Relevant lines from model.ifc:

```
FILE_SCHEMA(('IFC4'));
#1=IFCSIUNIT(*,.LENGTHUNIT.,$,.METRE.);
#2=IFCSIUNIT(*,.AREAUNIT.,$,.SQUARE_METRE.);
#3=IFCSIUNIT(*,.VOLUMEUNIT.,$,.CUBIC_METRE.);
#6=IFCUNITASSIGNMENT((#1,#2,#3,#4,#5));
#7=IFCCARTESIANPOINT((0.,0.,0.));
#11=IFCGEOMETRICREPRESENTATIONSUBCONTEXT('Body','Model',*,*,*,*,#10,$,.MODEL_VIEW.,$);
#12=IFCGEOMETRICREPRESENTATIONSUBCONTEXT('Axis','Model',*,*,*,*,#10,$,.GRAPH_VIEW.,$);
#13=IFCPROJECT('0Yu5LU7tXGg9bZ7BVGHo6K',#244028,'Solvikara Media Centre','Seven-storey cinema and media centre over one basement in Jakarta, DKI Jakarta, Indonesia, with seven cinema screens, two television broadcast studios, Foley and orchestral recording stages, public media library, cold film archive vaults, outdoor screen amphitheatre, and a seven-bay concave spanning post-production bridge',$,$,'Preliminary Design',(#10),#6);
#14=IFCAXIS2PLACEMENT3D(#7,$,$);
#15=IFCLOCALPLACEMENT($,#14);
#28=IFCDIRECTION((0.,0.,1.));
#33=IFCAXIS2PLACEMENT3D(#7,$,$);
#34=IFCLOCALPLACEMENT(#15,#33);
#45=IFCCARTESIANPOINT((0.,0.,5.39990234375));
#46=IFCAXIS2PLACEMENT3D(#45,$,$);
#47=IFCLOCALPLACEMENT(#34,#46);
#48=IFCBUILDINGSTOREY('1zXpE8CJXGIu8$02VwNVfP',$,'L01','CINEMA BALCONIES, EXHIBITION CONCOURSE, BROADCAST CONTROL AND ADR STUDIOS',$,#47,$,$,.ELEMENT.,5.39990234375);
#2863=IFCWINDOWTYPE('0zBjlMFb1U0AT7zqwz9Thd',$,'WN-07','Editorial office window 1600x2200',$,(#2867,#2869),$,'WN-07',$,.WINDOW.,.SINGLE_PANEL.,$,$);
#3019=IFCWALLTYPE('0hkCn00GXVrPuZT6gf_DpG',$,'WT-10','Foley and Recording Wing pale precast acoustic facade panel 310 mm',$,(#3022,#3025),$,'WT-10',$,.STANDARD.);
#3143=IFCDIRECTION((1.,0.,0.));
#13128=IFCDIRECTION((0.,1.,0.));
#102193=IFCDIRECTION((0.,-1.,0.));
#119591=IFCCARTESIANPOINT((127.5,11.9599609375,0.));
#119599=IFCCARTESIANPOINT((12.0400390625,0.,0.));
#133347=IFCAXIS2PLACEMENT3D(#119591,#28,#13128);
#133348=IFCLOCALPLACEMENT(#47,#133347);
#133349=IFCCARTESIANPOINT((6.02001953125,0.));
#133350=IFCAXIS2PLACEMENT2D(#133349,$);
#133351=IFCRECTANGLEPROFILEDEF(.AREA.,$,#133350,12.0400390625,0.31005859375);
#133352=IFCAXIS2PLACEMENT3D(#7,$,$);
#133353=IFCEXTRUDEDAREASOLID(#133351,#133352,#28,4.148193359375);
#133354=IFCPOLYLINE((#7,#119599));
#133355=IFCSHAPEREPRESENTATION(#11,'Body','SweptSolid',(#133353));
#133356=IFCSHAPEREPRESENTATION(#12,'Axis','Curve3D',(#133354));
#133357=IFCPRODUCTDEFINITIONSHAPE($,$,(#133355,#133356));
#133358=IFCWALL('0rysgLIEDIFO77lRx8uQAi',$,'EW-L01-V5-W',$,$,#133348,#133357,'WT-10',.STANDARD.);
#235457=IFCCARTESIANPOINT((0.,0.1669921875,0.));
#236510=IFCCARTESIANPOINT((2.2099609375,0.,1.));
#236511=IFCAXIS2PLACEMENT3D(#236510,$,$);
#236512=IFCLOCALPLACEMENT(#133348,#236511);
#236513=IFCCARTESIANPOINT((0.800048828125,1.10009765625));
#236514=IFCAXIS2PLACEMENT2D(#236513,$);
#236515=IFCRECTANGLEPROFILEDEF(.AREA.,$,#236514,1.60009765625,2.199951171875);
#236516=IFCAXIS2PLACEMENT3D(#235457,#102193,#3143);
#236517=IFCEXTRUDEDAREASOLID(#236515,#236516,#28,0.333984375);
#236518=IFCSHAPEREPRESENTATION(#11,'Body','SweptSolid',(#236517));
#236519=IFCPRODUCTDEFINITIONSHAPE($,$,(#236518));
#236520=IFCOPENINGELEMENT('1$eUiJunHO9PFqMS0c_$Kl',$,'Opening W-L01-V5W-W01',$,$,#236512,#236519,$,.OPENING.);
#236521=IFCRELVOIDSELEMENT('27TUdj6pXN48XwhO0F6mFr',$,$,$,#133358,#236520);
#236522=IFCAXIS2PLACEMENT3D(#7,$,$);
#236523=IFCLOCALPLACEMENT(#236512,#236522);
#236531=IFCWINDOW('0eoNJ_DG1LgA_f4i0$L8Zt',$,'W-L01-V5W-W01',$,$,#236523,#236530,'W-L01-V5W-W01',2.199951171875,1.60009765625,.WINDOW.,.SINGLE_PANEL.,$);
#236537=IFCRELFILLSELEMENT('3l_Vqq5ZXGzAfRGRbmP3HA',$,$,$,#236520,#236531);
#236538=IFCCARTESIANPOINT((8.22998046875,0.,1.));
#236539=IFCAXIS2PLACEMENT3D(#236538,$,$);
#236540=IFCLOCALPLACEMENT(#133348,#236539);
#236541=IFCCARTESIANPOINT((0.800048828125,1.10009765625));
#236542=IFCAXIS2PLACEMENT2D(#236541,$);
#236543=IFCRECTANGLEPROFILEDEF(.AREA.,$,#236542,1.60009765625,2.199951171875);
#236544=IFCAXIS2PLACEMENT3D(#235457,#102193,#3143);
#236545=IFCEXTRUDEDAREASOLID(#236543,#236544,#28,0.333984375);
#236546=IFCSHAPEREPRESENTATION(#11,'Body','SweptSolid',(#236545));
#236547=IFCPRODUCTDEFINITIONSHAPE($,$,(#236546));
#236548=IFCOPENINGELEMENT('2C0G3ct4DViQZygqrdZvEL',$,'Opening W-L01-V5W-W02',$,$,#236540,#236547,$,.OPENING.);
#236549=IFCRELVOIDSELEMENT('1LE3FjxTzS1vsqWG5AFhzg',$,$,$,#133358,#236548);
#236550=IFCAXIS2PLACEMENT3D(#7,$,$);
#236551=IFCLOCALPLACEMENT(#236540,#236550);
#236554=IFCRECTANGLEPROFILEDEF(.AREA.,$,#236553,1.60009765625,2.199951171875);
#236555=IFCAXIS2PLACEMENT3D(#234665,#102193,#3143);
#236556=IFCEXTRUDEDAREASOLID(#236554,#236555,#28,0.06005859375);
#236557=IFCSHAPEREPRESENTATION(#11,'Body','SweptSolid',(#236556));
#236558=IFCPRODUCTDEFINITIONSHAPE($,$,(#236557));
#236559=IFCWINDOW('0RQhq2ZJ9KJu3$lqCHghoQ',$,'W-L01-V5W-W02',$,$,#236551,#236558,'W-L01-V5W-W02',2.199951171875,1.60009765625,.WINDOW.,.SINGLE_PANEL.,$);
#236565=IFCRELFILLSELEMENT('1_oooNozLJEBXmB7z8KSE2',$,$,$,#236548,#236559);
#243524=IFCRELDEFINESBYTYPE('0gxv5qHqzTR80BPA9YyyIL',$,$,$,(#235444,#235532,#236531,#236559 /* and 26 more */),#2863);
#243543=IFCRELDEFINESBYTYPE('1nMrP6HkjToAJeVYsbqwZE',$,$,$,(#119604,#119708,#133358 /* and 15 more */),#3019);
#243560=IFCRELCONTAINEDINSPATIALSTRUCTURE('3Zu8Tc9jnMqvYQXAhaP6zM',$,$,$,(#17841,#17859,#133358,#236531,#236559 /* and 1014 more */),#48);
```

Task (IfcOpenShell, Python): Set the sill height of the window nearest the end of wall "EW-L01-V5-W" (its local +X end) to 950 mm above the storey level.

```python
import numpy as np
import ifcopenshell
import ifcopenshell.api.geometry
import ifcopenshell.geom
import ifcopenshell.util.element
import ifcopenshell.util.placement
import ifcopenshell.util.shape
import ifcopenshell.util.unit

model = ifcopenshell.open("model.ifc")
unit_scale = ifcopenshell.util.unit.calculate_unit_scale(model)

window = model.by_guid("0RQhq2ZJ9KJu3$lqCHghoQ")
opening = window.FillsVoids[0].RelatingOpeningElement
storey = ifcopenshell.util.element.get_container(window, ifc_class="IfcBuildingStorey")
level = ifcopenshell.util.placement.get_local_placement(storey.ObjectPlacement)[2, 3]

# The opening's origin need not be at the sill, so measure its lowest point.
shape = ifcopenshell.geom.create_shape(ifcopenshell.geom.settings(), opening)
bottom = ifcopenshell.util.shape.get_shape_bottom_elevation(shape, shape.geometry) / unit_scale
dz = level + 0.95 / unit_scale - bottom

shift = np.array([0.0, 0.0, dz])
# The window is placed relative to its opening, so it follows when the opening moves.
matrix = ifcopenshell.util.placement.get_local_placement(opening.ObjectPlacement)
matrix[:3, 3] += shift
ifcopenshell.api.geometry.edit_object_placement(
    model, product=opening, matrix=matrix, is_si=False, should_transform_children=True
)

print(f"moved by {dz * unit_scale:+.3f} m")

model.write("model_edited.ifc")
```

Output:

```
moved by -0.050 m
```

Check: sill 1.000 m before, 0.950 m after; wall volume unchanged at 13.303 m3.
